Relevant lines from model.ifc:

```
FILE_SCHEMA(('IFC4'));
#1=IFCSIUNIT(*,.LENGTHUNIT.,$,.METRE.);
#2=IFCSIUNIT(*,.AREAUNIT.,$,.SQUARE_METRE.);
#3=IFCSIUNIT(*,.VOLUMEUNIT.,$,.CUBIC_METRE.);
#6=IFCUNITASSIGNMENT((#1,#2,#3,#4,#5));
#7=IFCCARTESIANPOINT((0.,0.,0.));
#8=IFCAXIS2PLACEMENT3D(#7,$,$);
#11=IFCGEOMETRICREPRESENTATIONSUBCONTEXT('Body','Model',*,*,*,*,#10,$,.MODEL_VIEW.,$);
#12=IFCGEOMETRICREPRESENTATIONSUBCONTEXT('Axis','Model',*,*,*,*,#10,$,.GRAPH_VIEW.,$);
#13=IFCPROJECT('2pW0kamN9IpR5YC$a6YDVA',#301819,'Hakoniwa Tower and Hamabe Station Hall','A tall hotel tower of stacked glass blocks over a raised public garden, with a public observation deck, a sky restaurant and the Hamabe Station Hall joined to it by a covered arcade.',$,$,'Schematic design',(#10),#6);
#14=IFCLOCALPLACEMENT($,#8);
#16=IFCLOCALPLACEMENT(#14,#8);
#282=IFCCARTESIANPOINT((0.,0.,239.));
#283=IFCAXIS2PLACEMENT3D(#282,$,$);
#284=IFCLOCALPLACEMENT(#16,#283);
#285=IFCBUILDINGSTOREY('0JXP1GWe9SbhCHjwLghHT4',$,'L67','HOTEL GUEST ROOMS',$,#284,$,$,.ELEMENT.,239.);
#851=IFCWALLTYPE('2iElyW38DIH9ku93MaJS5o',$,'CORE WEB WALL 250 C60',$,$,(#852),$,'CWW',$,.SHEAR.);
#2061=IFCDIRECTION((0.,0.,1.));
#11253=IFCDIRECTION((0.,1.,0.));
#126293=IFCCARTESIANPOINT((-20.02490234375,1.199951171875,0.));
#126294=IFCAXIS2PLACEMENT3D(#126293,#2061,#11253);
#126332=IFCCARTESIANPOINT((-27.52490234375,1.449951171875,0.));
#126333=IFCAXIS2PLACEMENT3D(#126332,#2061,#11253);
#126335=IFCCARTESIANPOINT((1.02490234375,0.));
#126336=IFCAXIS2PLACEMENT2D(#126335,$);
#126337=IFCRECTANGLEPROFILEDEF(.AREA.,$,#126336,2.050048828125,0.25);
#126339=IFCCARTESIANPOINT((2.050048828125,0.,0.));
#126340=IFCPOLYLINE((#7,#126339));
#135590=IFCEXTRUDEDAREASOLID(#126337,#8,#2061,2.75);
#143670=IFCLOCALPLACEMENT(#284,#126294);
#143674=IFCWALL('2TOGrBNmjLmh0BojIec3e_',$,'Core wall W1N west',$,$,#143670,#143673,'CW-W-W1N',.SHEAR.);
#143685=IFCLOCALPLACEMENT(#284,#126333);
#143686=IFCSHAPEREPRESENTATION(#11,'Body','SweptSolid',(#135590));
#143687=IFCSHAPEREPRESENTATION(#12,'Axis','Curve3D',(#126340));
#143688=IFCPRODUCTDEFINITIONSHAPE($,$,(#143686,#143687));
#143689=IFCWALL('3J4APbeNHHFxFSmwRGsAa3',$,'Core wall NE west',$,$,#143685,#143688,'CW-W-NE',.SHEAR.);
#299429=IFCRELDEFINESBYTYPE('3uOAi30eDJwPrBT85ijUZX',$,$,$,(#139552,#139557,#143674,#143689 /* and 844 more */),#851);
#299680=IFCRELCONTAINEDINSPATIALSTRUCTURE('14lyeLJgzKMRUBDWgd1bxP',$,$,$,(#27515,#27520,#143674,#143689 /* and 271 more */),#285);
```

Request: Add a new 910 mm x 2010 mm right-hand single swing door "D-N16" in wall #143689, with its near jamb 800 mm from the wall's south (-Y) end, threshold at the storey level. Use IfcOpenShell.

```python
import numpy as np
import ifcopenshell
import ifcopenshell.api.feature
import ifcopenshell.api.geometry
import ifcopenshell.api.root
import ifcopenshell.api.spatial
import ifcopenshell.geom
import ifcopenshell.util.element
import ifcopenshell.util.placement
import ifcopenshell.util.representation
import ifcopenshell.util.shape
import ifcopenshell.util.unit

model = ifcopenshell.open("model.ifc")
unit_scale = ifcopenshell.util.unit.calculate_unit_scale(model)
settings = ifcopenshell.geom.settings()


def volume(element):
    """Net volume in cubic metres, openings subtracted."""
    shape = ifcopenshell.geom.create_shape(settings, element)
    return ifcopenshell.util.shape.get_volume(shape.geometry)


wall = model.by_id(143689)
storey = ifcopenshell.util.element.get_container(wall, ifc_class="IfcBuildingStorey")
context = ifcopenshell.util.representation.get_context(model, "Model", "Body", "MODEL_VIEW")
before = volume(wall)

width, height, from_end, sill = 0.91, 2.01, 0.8, 0.0  # metres

# The wall runs along its own X axis, and the end named is its -X end.
wall_shape = ifcopenshell.geom.create_shape(settings, wall)
x, y, z = ifcopenshell.util.shape.get_vertices(wall_shape.geometry).T
start = x.min() + from_end
face, thickness = float(y.min()), float(y.max() - y.min())
wall_matrix = ifcopenshell.util.placement.get_local_placement(wall.ObjectPlacement)
level = ifcopenshell.util.placement.get_local_placement(storey.ObjectPlacement)[2, 3]


def in_wall(x, y):
    """Placement at x, y metres in the wall's axes, at sill height."""
    matrix = wall_matrix.copy()
    matrix[:, 3] = wall_matrix @ np.array([x / unit_scale, y / unit_scale, 0.0, 1.0])
    matrix[2, 3] = level + sill / unit_scale
    return matrix


# Opening: a box that overshoots both wall faces by 50 mm.
opening = ifcopenshell.api.root.create_entity(model, ifc_class="IfcOpeningElement", predefined_type="OPENING")
box = ifcopenshell.api.geometry.add_wall_representation(
    model, context=context, length=width, height=height, thickness=thickness + 0.1
)
ifcopenshell.api.geometry.assign_representation(model, product=opening, representation=box)
ifcopenshell.api.geometry.edit_object_placement(model, product=opening, matrix=in_wall(start, face - 0.05), is_si=False)
ifcopenshell.api.feature.add_feature(model, feature=opening, element=wall)

door = ifcopenshell.api.root.create_entity(model, ifc_class="IfcDoor", name="D-N16", predefined_type="DOOR")
door.OverallWidth, door.OverallHeight = width / unit_scale, height / unit_scale
door.OperationType = "SINGLE_SWING_RIGHT"
body = ifcopenshell.api.geometry.add_door_representation(
    model,
    context=context,
    overall_width=door.OverallWidth,
    overall_height=door.OverallHeight,
    operation_type="SINGLE_SWING_RIGHT",
    lining_properties={"LiningDepth": thickness / unit_scale, "ThresholdDepth": thickness / unit_scale},
)
ifcopenshell.api.geometry.assign_representation(model, product=door, representation=body)
ifcopenshell.api.spatial.assign_container(model, products=[door], relating_structure=storey)
ifcopenshell.api.feature.add_filling(model, opening=opening, element=door)

# The lining spans the wall, so the door starts at the wall face.
ifcopenshell.api.geometry.edit_object_placement(model, product=door, matrix=in_wall(start, face), is_si=False)

after = volume(wall)

print(f"wall volume {before:.3f} -> {after:.3f} m3")

model.write("model_rev.ifc")
```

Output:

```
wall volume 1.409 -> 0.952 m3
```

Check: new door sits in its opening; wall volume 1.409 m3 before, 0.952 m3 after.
